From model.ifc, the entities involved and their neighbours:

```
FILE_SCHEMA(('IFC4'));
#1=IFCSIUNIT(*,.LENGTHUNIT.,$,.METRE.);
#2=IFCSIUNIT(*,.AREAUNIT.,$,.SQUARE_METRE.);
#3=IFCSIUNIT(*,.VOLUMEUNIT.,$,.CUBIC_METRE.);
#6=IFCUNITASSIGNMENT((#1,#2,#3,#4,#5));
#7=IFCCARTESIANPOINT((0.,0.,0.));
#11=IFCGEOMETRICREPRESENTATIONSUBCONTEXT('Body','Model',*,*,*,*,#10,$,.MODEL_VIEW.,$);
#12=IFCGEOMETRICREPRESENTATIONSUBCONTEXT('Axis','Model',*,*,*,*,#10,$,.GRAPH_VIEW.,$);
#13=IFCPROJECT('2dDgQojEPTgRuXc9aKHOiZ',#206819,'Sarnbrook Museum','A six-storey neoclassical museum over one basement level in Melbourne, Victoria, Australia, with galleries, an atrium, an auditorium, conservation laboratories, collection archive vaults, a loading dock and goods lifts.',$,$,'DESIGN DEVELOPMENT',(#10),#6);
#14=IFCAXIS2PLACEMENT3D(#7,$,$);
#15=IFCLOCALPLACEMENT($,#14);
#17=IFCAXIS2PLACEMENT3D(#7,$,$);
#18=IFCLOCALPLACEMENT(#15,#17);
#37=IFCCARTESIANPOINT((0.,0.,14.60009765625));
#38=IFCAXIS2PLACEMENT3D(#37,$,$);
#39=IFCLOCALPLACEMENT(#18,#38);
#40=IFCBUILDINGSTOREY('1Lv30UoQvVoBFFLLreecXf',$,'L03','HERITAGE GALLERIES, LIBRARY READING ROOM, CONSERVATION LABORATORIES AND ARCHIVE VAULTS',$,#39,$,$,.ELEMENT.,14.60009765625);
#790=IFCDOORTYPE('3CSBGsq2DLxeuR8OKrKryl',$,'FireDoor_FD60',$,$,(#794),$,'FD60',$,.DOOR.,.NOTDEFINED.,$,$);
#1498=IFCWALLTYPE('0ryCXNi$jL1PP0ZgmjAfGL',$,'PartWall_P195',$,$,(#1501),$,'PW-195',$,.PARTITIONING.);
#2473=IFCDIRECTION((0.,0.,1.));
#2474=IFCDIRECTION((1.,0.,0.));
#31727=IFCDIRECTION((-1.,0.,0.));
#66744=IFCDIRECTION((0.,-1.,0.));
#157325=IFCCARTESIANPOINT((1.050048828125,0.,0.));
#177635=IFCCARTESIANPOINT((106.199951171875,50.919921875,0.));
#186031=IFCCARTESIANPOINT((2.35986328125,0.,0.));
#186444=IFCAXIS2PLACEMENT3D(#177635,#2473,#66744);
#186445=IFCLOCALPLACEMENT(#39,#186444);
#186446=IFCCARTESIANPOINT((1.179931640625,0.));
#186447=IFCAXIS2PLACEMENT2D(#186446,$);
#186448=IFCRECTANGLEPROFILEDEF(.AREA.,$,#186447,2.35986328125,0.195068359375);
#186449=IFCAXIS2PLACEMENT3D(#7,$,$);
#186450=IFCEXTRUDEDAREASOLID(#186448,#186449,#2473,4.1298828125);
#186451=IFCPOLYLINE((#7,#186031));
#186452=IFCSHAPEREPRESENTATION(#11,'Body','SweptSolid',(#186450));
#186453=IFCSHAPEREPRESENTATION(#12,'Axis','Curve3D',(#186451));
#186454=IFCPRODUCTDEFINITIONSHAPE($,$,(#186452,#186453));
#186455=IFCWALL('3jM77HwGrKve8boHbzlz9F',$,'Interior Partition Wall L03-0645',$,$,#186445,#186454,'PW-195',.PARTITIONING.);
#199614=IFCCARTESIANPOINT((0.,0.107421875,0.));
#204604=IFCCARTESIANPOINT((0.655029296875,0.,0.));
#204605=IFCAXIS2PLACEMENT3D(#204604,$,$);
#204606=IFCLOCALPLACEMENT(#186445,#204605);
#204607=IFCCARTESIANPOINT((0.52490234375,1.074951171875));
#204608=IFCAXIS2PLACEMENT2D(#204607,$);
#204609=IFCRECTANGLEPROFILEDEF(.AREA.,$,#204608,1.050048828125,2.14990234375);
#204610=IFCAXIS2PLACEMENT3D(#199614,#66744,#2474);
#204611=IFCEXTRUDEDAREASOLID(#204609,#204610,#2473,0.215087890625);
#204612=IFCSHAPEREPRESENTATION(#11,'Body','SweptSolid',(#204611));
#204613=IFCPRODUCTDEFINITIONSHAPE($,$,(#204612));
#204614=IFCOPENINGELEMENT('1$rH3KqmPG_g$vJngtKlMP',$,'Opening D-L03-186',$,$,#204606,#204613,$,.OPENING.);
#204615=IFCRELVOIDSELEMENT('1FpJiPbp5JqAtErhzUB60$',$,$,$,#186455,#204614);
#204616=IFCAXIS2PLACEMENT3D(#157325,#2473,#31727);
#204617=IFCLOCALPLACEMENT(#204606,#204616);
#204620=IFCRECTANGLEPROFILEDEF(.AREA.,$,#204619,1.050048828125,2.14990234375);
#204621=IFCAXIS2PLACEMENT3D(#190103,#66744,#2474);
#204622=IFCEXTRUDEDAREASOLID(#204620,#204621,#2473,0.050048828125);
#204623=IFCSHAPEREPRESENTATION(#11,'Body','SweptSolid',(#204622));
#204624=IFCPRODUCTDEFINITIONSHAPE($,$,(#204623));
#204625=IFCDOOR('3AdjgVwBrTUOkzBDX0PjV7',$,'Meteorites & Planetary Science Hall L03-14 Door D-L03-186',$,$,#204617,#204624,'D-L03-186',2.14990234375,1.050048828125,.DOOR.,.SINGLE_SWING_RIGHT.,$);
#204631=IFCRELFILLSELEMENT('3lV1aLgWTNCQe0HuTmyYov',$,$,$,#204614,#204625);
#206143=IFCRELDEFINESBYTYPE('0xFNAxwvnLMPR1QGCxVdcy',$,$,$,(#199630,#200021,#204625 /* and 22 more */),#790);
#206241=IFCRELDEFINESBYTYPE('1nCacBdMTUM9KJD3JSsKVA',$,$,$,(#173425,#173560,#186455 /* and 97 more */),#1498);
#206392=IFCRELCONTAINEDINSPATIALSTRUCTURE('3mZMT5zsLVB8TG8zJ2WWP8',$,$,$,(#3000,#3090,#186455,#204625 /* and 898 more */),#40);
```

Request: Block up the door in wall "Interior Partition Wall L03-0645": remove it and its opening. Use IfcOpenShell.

```python
import ifcopenshell
import ifcopenshell.api.feature
import ifcopenshell.api.root
import ifcopenshell.geom
import ifcopenshell.util.shape

model = ifcopenshell.open("model.ifc")
settings = ifcopenshell.geom.settings()


def volume(element):
    """Net volume in cubic metres, openings subtracted."""
    shape = ifcopenshell.geom.create_shape(settings, element)
    return ifcopenshell.util.shape.get_volume(shape.geometry)


door = model.by_id(204625)
opening = door.FillsVoids[0].RelatingOpeningElement
wall = opening.VoidsElements[0].RelatingBuildingElement
before = volume(wall)

ifcopenshell.api.root.remove_product(model, product=door)
ifcopenshell.api.feature.remove_feature(model, feature=opening)

after = volume(wall)

print(f"wall volume {before:.3f} -> {after:.3f} m3")

model.write("model_rev.ifc")
```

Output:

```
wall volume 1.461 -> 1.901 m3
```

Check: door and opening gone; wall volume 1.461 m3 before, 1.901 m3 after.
